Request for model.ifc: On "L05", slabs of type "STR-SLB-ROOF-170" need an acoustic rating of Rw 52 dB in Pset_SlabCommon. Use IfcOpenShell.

First a look at what the model holds.

```python
import ifcopenshell
import ifcopenshell.util.element

model = ifcopenshell.open("model.ifc")
print(model.schema)
storey = next(s for s in model.by_type("IfcBuildingStorey") if s.Name == "L05")
slabs = [e for e in ifcopenshell.util.element.get_decomposition(storey) if e.is_a("IfcSlab")]
seen = {}
for e in slabs:
    element_type = ifcopenshell.util.element.get_type(e)
    key = (element_type.Name if element_type != e and element_type else None, ifcopenshell.util.element.get_pset(e, "Pset_SlabCommon", "AcousticRating"))
    seen[key] = seen.get(key, 0) + 1
for (name, value), count in sorted(seen.items(), key=str):
    print(count, "x", name, "|", value)
```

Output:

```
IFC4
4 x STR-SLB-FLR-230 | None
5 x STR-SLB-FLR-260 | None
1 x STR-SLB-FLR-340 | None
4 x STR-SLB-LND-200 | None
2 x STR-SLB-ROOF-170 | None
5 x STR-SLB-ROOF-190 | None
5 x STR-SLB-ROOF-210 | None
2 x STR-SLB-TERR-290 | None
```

```python
import ifcopenshell
import ifcopenshell.api.pset
import ifcopenshell.util.element

model = ifcopenshell.open("model.ifc")

storey = next(s for s in model.by_type("IfcBuildingStorey") if s.Name == "L05")
slabs = [e for e in ifcopenshell.util.element.get_decomposition(storey) if e.is_a("IfcSlab")]

count = 0
for e in slabs:
    element_type = ifcopenshell.util.element.get_type(e)
    if element_type in (None, e) or element_type.Name != "STR-SLB-ROOF-170":
        continue
    # add_pset returns the element's existing set when there is one.
    pset = ifcopenshell.api.pset.add_pset(model, product=e, name="Pset_SlabCommon")
    ifcopenshell.api.pset.edit_pset(model, pset=pset, properties={"AcousticRating": "Rw 52 dB"})
    count += 1

print(count, "slabs updated")

model.write("model-out.ifc")
```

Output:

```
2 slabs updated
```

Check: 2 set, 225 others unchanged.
